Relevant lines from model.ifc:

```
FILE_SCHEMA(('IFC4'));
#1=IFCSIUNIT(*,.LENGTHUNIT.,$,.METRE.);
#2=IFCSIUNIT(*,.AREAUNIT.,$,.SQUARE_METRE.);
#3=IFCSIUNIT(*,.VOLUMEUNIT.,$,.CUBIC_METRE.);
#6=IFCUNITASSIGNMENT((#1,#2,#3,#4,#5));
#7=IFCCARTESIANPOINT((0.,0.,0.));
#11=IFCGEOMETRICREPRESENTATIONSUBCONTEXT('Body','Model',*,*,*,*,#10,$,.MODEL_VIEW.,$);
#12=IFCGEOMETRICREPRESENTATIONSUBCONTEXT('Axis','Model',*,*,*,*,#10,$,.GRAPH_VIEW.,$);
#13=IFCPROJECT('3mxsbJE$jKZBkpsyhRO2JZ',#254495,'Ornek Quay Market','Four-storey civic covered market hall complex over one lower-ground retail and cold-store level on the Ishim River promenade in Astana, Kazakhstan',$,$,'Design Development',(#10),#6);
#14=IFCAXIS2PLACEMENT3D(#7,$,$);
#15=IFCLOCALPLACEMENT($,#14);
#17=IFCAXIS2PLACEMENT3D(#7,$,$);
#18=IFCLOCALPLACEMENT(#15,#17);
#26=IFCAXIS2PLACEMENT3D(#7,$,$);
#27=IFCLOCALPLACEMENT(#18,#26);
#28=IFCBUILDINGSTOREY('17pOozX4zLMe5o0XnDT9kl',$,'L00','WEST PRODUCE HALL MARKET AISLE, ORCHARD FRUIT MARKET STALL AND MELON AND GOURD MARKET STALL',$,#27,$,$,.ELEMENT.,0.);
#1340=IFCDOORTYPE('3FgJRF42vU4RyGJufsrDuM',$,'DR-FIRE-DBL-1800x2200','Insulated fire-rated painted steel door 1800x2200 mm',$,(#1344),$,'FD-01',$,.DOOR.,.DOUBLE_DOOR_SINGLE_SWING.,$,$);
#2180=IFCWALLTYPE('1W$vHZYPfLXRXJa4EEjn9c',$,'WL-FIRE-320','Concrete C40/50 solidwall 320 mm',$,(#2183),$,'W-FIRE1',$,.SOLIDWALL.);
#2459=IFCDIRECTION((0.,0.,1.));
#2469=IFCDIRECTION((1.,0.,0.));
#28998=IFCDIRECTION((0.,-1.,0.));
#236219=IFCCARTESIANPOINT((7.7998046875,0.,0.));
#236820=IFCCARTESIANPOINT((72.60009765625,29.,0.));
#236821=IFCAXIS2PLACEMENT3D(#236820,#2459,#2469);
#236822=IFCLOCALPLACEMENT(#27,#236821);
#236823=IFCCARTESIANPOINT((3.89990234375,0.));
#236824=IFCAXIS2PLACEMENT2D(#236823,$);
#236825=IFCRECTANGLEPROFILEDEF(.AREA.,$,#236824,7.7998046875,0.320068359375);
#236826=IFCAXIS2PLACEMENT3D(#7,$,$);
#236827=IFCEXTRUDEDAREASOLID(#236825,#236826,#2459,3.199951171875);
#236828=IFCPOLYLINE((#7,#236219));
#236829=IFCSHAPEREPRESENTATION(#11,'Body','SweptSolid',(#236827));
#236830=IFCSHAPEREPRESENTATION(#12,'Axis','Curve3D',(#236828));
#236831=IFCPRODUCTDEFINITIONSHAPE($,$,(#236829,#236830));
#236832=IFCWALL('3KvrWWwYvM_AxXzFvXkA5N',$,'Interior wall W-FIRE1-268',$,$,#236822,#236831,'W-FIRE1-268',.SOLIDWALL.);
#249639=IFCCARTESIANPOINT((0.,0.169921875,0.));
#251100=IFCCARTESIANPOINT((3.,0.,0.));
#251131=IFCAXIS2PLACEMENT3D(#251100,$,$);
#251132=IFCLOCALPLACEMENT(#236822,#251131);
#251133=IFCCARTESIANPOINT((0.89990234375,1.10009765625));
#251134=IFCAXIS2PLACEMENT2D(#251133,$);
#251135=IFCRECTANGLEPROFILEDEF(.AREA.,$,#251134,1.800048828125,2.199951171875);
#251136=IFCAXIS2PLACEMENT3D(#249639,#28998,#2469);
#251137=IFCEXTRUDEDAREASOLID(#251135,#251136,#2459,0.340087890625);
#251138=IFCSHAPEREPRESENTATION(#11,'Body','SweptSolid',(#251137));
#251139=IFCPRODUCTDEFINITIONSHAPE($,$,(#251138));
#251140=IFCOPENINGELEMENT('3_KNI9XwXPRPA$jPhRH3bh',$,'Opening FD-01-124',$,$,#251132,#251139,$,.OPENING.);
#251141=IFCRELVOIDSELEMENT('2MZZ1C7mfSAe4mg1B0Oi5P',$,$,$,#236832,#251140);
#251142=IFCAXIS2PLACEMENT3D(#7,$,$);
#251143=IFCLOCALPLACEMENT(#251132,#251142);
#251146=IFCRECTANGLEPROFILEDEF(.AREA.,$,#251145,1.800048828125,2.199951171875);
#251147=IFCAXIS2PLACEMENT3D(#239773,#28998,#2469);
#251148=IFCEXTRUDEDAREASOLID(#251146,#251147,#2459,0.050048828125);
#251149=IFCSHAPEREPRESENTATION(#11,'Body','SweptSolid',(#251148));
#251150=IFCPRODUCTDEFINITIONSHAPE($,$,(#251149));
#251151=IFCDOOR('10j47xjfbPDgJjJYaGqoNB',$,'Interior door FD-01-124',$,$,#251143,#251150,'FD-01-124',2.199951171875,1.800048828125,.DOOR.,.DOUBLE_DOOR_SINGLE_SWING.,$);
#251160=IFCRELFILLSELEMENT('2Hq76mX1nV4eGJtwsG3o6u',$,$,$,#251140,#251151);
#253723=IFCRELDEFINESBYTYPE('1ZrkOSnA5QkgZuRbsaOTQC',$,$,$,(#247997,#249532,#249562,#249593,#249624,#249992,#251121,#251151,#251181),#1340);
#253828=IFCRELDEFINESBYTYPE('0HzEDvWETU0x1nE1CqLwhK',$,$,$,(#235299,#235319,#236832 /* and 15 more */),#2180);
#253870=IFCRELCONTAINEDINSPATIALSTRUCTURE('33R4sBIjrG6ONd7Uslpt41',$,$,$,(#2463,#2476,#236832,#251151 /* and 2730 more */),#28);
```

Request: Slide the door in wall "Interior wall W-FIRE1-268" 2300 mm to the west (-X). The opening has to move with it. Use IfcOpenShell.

```python
import ifcopenshell
import ifcopenshell.api.geometry
import ifcopenshell.util.placement
import ifcopenshell.util.unit

model = ifcopenshell.open("model.ifc")
unit_scale = ifcopenshell.util.unit.calculate_unit_scale(model)

door = model.by_guid("10j47xjfbPDgJjJYaGqoNB")
opening = door.FillsVoids[0].RelatingOpeningElement
wall = opening.VoidsElements[0].RelatingBuildingElement

wall_matrix = ifcopenshell.util.placement.get_local_placement(wall.ObjectPlacement)
shift = wall_matrix[:3, 0] * -2.3 / unit_scale
before = ifcopenshell.util.placement.get_local_placement(door.ObjectPlacement)[:3, 3].copy()

# The door is placed relative to its opening, so it follows when the opening moves.
matrix = ifcopenshell.util.placement.get_local_placement(opening.ObjectPlacement)
matrix[:3, 3] += shift
ifcopenshell.api.geometry.edit_object_placement(
    model, product=opening, matrix=matrix, is_si=False, should_transform_children=True
)

after = ifcopenshell.util.placement.get_local_placement(door.ObjectPlacement)[:3, 3]
print("door moved by", (after - before).round(3) + 0.0)

model.write("model-out.ifc")
```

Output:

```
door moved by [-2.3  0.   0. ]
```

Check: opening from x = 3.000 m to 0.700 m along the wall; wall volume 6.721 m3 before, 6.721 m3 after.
